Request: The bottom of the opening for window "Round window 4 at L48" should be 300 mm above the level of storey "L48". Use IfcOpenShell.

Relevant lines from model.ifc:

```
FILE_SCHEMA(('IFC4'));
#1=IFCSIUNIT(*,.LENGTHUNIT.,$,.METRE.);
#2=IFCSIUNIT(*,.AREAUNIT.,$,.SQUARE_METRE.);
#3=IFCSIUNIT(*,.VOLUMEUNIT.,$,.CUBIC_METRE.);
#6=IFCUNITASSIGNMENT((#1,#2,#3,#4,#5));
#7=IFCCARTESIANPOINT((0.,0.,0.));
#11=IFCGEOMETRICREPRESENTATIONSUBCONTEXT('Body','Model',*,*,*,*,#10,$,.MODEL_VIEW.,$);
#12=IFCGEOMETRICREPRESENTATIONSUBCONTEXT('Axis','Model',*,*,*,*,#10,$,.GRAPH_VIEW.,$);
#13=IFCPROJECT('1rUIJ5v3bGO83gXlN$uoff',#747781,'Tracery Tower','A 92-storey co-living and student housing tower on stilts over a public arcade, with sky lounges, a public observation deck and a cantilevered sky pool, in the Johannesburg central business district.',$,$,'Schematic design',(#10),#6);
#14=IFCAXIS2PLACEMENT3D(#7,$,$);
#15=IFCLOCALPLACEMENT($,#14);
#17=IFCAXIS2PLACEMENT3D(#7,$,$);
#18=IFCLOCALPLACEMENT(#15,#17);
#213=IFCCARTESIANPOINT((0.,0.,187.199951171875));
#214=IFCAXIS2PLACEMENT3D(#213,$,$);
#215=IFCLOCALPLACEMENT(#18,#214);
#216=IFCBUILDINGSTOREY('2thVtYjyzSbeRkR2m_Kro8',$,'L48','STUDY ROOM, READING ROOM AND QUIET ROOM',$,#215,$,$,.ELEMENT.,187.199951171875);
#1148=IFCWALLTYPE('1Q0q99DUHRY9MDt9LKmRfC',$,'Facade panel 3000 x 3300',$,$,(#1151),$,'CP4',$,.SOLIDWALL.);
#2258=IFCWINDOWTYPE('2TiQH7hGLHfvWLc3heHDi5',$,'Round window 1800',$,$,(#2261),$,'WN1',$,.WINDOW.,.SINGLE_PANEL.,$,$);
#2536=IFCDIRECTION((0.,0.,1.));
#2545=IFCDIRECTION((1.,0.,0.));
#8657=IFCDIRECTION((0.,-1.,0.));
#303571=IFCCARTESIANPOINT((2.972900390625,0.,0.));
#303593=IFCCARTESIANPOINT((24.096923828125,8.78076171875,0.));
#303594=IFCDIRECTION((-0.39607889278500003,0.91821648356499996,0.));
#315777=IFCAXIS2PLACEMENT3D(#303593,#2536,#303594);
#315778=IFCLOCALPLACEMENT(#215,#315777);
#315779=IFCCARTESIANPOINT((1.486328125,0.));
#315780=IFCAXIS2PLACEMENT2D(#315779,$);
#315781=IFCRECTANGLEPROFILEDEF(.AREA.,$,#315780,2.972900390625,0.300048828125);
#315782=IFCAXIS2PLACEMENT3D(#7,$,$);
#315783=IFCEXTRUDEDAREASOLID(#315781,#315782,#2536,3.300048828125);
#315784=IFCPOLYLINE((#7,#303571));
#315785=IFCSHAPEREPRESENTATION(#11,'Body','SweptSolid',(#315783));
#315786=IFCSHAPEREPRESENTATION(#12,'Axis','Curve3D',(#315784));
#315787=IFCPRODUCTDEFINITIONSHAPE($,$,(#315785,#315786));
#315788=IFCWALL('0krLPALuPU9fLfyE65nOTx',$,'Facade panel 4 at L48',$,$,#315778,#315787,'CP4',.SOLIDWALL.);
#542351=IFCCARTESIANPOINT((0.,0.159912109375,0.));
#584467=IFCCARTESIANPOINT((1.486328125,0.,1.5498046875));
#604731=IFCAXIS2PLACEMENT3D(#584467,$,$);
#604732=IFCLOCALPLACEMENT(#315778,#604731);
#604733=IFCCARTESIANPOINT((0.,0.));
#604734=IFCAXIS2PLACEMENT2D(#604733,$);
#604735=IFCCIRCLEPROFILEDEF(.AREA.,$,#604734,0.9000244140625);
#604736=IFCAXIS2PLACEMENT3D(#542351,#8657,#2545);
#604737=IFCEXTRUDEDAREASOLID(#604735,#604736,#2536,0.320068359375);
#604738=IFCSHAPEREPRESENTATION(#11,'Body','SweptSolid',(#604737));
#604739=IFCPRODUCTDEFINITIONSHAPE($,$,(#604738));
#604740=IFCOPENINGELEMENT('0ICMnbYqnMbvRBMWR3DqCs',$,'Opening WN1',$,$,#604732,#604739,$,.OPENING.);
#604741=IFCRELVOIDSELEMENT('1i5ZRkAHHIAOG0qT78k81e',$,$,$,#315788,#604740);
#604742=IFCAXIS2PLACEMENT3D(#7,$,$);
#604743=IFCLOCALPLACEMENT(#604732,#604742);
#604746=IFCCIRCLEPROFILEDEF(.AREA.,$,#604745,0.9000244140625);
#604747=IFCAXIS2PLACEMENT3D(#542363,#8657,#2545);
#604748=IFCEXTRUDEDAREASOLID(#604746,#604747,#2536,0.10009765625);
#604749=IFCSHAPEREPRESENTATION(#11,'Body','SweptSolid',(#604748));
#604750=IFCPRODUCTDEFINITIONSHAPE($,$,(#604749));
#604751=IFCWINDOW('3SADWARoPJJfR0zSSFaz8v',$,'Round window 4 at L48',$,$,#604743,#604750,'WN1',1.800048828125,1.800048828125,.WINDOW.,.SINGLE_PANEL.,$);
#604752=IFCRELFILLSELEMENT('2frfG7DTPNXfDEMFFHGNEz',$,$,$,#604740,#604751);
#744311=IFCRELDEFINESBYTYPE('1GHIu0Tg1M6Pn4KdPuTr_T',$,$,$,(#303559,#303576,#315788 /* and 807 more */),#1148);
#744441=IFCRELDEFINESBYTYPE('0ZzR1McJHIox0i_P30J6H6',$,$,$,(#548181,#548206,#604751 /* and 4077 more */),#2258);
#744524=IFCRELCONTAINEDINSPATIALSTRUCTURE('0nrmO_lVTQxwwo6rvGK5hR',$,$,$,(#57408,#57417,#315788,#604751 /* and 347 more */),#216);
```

```python
import numpy as np
import ifcopenshell
import ifcopenshell.api.geometry
import ifcopenshell.geom
import ifcopenshell.util.element
import ifcopenshell.util.placement
import ifcopenshell.util.shape
import ifcopenshell.util.unit

model = ifcopenshell.open("model.ifc")
unit_scale = ifcopenshell.util.unit.calculate_unit_scale(model)

window = model.by_id(604751)
opening = window.FillsVoids[0].RelatingOpeningElement
storey = ifcopenshell.util.element.get_container(window, ifc_class="IfcBuildingStorey")
level = ifcopenshell.util.placement.get_local_placement(storey.ObjectPlacement)[2, 3]

# The opening's origin need not be at the sill, so measure its lowest point.
shape = ifcopenshell.geom.create_shape(ifcopenshell.geom.settings(), opening)
bottom = ifcopenshell.util.shape.get_shape_bottom_elevation(shape, shape.geometry) / unit_scale
dz = level + 0.3 / unit_scale - bottom

shift = np.array([0.0, 0.0, dz])
# The window is placed relative to its opening, so it follows when the opening moves.
matrix = ifcopenshell.util.placement.get_local_placement(opening.ObjectPlacement)
matrix[:3, 3] += shift
ifcopenshell.api.geometry.edit_object_placement(
    model, product=opening, matrix=matrix, is_si=False, should_transform_children=True
)

print(f"moved by {dz * unit_scale:+.3f} m")

model.write("model_edited.ifc")
```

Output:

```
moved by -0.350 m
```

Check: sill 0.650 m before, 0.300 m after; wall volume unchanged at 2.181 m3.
